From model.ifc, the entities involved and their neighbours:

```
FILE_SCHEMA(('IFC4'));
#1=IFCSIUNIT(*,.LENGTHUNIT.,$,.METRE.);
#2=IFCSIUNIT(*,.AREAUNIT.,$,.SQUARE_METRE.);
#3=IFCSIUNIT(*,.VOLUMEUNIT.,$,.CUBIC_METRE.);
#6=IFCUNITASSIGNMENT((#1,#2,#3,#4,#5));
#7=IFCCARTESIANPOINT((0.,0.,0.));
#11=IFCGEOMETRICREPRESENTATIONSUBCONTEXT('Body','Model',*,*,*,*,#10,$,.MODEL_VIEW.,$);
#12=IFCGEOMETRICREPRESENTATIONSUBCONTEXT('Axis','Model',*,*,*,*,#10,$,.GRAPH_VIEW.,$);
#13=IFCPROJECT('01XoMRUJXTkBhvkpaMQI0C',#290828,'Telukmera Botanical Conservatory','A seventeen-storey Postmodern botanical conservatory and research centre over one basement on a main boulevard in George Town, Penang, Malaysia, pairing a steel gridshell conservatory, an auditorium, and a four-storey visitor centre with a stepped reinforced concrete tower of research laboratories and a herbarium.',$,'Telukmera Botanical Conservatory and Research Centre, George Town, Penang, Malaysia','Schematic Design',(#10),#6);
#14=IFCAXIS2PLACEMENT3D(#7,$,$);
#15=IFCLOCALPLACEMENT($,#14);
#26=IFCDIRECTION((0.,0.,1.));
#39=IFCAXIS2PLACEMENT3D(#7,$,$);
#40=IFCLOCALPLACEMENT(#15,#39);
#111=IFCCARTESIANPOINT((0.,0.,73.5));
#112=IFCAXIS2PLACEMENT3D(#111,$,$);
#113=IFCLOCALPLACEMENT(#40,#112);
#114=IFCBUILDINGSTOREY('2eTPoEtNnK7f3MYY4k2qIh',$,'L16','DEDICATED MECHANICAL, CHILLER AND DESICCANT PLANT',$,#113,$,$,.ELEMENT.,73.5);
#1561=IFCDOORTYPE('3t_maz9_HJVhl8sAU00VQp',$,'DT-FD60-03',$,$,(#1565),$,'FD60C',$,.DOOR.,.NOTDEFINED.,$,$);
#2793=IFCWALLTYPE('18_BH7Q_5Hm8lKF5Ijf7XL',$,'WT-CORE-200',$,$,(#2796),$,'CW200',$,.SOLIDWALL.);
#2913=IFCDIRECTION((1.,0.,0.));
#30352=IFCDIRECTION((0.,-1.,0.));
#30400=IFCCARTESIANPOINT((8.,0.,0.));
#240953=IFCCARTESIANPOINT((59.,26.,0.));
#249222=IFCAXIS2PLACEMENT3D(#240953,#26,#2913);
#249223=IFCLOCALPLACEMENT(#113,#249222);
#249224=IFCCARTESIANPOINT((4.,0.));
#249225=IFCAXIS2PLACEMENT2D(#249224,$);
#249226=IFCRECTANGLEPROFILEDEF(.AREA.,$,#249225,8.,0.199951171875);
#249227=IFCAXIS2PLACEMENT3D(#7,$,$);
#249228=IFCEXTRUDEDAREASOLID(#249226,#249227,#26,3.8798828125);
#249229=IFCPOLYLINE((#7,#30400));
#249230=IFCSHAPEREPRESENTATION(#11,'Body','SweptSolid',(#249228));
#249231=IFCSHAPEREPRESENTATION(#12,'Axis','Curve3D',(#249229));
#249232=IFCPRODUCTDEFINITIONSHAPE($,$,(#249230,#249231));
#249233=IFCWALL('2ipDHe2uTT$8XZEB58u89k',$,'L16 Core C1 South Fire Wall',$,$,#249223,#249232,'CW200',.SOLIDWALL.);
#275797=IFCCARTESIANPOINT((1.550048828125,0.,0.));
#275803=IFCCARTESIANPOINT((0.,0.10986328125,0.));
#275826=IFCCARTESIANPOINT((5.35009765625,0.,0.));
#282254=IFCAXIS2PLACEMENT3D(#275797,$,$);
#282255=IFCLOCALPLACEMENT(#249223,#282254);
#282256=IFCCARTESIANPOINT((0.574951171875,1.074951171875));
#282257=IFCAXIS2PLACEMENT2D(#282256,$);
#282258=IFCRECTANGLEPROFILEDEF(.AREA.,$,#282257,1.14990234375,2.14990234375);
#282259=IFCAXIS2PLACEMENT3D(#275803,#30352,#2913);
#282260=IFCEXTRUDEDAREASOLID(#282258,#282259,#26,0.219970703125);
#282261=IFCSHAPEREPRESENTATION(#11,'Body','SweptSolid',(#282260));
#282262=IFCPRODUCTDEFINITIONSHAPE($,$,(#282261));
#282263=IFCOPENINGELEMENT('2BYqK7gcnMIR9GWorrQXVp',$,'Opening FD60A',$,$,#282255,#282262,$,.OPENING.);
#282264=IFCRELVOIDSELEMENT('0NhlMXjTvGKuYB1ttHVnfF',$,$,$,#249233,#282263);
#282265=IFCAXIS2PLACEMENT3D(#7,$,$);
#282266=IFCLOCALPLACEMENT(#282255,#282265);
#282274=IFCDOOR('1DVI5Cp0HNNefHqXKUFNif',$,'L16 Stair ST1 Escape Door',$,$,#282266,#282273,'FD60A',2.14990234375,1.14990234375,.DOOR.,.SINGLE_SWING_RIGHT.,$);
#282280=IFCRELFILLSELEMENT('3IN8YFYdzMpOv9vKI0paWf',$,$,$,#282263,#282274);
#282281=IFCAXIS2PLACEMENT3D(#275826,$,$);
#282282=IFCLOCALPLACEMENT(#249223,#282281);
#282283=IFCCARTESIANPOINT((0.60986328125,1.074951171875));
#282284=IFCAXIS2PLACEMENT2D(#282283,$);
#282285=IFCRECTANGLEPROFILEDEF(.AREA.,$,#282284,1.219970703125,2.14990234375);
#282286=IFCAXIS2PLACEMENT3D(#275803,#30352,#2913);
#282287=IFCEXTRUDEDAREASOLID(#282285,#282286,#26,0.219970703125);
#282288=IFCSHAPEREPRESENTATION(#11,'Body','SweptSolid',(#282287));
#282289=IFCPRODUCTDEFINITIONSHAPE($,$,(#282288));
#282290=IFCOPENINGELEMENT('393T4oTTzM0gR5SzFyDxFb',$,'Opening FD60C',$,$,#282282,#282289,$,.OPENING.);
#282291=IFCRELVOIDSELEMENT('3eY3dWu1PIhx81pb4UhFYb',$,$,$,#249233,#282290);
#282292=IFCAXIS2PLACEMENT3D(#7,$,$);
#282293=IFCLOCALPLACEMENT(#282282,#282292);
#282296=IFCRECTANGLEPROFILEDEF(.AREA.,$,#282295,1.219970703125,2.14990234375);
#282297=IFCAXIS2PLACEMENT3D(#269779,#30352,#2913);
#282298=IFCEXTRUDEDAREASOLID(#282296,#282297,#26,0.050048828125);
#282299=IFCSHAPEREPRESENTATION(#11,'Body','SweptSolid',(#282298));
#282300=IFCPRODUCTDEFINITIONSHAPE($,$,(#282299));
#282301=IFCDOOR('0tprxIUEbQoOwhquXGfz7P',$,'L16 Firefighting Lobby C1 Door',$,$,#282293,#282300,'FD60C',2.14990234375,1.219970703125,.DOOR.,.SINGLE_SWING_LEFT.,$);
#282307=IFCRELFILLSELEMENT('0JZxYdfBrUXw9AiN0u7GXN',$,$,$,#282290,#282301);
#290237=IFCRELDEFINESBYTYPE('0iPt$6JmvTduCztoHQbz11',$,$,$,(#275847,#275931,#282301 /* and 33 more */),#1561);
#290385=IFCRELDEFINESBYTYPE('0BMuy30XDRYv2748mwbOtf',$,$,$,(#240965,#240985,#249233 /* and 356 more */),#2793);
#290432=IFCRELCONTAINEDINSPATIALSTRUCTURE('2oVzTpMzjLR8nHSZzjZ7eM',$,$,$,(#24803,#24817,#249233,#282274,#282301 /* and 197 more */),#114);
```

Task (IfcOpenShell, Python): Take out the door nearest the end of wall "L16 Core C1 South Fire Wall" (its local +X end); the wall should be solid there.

```python
import ifcopenshell
import ifcopenshell.api.feature
import ifcopenshell.api.root
import ifcopenshell.geom
import ifcopenshell.util.shape

model = ifcopenshell.open("model.ifc")
settings = ifcopenshell.geom.settings()


def volume(element):
    """Net volume in cubic metres, openings subtracted."""
    shape = ifcopenshell.geom.create_shape(settings, element)
    return ifcopenshell.util.shape.get_volume(shape.geometry)


door = model.by_id(282301)
opening = door.FillsVoids[0].RelatingOpeningElement
wall = opening.VoidsElements[0].RelatingBuildingElement
before = volume(wall)

ifcopenshell.api.root.remove_product(model, product=door)
ifcopenshell.api.feature.remove_feature(model, feature=opening)

after = volume(wall)

print(f"wall volume {before:.3f} -> {after:.3f} m3")

model.write("model_updated.ifc")
```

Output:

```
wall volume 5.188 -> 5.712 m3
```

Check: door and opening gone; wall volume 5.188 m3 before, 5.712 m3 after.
